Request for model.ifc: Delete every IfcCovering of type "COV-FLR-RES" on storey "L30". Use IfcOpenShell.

First a look at what the model holds.

```python
import ifcopenshell
import ifcopenshell.util.element

model = ifcopenshell.open("model.ifc")
print(model.schema)
storey = next(s for s in model.by_type("IfcBuildingStorey") if s.Name == "L30")
coverings = [e for e in ifcopenshell.util.element.get_decomposition(storey) if e.is_a("IfcCovering")]
seen = {}
for e in coverings:
    element_type = ifcopenshell.util.element.get_type(e)
    name = element_type.Name if element_type not in (None, e) else None
    seen[name] = seen.get(name, 0) + 1
for name, count in sorted(seen.items(), key=str):
    print(count, "x", name)
```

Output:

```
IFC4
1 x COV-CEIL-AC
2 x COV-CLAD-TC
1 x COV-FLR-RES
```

```python
import ifcopenshell
import ifcopenshell.api.root
import ifcopenshell.util.element

model = ifcopenshell.open("model.ifc")

storey = next(s for s in model.by_type("IfcBuildingStorey") if s.Name == "L30")
coverings = [e for e in ifcopenshell.util.element.get_decomposition(storey) if e.is_a("IfcCovering")]
targets = [e for e in coverings if (t := ifcopenshell.util.element.get_type(e)) not in (None, e) and t.Name == "COV-FLR-RES"]

for e in targets:
    ifcopenshell.api.root.remove_product(model, product=e)
print(len(targets), "removed")

model.write("model-out.ifc")
```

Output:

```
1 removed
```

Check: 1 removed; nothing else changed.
